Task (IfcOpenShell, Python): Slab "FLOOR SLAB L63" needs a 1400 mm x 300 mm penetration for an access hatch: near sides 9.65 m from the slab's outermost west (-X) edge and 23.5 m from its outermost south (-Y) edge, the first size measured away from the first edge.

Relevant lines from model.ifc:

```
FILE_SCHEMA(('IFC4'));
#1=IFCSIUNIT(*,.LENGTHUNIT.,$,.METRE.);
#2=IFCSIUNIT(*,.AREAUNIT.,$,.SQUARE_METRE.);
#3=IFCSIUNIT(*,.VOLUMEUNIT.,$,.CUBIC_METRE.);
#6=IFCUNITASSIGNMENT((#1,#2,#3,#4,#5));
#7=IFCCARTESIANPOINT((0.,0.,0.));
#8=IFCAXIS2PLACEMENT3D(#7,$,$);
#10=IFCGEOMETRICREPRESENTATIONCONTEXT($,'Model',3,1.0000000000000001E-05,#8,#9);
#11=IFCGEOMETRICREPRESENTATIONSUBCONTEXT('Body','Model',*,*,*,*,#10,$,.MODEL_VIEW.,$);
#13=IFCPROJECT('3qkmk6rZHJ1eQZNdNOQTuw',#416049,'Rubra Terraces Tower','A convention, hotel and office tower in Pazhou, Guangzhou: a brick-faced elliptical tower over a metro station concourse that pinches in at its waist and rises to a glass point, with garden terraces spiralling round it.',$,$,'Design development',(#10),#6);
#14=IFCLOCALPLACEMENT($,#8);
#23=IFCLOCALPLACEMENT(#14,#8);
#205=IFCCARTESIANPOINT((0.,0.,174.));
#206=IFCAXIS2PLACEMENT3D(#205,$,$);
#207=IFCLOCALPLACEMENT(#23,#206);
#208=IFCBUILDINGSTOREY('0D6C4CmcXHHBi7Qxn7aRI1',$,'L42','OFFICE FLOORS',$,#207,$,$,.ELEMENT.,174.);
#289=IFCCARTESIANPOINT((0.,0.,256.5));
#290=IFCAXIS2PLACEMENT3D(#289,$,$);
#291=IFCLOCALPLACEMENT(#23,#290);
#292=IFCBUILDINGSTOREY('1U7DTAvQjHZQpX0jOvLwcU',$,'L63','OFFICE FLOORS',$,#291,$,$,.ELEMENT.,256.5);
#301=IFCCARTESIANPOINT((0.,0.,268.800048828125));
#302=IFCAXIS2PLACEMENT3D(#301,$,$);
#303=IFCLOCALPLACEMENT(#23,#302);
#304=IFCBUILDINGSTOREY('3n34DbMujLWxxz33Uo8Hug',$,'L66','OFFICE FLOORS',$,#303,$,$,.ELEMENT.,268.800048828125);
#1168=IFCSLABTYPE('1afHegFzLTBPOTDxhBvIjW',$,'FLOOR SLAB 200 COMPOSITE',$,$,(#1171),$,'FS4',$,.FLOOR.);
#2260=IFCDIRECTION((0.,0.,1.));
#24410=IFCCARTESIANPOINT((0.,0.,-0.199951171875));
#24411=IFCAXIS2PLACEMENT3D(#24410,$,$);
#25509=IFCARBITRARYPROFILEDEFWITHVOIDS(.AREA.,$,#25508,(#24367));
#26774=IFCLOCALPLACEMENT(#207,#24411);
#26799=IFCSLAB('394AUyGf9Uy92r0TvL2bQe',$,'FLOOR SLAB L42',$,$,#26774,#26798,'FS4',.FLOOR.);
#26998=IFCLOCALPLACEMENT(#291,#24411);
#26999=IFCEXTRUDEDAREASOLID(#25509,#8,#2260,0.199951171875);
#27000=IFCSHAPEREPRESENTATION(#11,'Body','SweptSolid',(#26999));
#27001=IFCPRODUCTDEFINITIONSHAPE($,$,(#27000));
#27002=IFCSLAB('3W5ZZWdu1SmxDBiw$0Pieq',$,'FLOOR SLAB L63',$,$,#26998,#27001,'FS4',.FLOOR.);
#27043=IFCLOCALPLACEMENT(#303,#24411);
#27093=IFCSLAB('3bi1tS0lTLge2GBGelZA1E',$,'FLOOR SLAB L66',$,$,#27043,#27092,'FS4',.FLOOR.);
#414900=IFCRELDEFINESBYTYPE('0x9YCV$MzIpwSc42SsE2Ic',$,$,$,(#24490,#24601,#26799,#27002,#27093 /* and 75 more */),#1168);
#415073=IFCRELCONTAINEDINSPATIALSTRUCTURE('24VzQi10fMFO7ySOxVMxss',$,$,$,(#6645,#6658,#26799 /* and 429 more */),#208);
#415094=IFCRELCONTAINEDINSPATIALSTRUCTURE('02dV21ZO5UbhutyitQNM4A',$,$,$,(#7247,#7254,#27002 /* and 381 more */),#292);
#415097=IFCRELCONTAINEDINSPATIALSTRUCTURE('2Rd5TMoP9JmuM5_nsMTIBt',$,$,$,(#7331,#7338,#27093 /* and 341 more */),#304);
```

```python
import numpy as np
import ifcopenshell
import ifcopenshell.api.feature
import ifcopenshell.api.geometry
import ifcopenshell.api.root
import ifcopenshell.geom
import ifcopenshell.util.placement
import ifcopenshell.util.representation
import ifcopenshell.util.shape
import ifcopenshell.util.unit

model = ifcopenshell.open("model.ifc")
unit_scale = ifcopenshell.util.unit.calculate_unit_scale(model)
settings = ifcopenshell.geom.settings()


def volume(element):
    """Net volume in cubic metres, openings subtracted."""
    shape = ifcopenshell.geom.create_shape(settings, element)
    return ifcopenshell.util.shape.get_volume(shape.geometry)


slab = model.by_guid("3W5ZZWdu1SmxDBiw$0Pieq")
before = volume(slab)

# Extent in the slab's own axes, in metres. The edges named are its -X and -Y sides.
slab_shape = ifcopenshell.geom.create_shape(settings, slab)
vertices = ifcopenshell.util.shape.get_vertices(slab_shape.geometry)
x_min, y_min, bottom = vertices.min(axis=0)
top = vertices[:, 2].max()

opening = ifcopenshell.api.root.create_entity(model, ifc_class="IfcOpeningElement", name="Access hatch opening", predefined_type="OPENING")
context = ifcopenshell.util.representation.get_context(model, "Model", "Body", "MODEL_VIEW")
width, depth = 1.4, 0.3
outline = [(0.0, 0.0), (width, 0.0), (width, depth), (0.0, depth), (0.0, 0.0)]
# Overshoot both faces by 50 mm so the cut is clean.
shape = ifcopenshell.api.geometry.add_slab_representation(
    model, context=context, depth=top - bottom + 0.1, polyline=outline
)
ifcopenshell.api.geometry.assign_representation(model, product=opening, representation=shape)

matrix = ifcopenshell.util.placement.get_local_placement(slab.ObjectPlacement)
matrix[:, 3] = matrix @ np.append(np.array([x_min + 9.65, y_min + 23.5, bottom - 0.05]) / unit_scale, 1.0)
ifcopenshell.api.geometry.edit_object_placement(model, product=opening, matrix=matrix, is_si=False)
ifcopenshell.api.feature.add_feature(model, feature=opening, element=slab)

after = volume(slab)

print(f"slab volume {before:.3f} -> {after:.3f} m3")

model.write("model-out.ifc")
```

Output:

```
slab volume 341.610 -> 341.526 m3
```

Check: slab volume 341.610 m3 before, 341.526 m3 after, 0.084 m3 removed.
